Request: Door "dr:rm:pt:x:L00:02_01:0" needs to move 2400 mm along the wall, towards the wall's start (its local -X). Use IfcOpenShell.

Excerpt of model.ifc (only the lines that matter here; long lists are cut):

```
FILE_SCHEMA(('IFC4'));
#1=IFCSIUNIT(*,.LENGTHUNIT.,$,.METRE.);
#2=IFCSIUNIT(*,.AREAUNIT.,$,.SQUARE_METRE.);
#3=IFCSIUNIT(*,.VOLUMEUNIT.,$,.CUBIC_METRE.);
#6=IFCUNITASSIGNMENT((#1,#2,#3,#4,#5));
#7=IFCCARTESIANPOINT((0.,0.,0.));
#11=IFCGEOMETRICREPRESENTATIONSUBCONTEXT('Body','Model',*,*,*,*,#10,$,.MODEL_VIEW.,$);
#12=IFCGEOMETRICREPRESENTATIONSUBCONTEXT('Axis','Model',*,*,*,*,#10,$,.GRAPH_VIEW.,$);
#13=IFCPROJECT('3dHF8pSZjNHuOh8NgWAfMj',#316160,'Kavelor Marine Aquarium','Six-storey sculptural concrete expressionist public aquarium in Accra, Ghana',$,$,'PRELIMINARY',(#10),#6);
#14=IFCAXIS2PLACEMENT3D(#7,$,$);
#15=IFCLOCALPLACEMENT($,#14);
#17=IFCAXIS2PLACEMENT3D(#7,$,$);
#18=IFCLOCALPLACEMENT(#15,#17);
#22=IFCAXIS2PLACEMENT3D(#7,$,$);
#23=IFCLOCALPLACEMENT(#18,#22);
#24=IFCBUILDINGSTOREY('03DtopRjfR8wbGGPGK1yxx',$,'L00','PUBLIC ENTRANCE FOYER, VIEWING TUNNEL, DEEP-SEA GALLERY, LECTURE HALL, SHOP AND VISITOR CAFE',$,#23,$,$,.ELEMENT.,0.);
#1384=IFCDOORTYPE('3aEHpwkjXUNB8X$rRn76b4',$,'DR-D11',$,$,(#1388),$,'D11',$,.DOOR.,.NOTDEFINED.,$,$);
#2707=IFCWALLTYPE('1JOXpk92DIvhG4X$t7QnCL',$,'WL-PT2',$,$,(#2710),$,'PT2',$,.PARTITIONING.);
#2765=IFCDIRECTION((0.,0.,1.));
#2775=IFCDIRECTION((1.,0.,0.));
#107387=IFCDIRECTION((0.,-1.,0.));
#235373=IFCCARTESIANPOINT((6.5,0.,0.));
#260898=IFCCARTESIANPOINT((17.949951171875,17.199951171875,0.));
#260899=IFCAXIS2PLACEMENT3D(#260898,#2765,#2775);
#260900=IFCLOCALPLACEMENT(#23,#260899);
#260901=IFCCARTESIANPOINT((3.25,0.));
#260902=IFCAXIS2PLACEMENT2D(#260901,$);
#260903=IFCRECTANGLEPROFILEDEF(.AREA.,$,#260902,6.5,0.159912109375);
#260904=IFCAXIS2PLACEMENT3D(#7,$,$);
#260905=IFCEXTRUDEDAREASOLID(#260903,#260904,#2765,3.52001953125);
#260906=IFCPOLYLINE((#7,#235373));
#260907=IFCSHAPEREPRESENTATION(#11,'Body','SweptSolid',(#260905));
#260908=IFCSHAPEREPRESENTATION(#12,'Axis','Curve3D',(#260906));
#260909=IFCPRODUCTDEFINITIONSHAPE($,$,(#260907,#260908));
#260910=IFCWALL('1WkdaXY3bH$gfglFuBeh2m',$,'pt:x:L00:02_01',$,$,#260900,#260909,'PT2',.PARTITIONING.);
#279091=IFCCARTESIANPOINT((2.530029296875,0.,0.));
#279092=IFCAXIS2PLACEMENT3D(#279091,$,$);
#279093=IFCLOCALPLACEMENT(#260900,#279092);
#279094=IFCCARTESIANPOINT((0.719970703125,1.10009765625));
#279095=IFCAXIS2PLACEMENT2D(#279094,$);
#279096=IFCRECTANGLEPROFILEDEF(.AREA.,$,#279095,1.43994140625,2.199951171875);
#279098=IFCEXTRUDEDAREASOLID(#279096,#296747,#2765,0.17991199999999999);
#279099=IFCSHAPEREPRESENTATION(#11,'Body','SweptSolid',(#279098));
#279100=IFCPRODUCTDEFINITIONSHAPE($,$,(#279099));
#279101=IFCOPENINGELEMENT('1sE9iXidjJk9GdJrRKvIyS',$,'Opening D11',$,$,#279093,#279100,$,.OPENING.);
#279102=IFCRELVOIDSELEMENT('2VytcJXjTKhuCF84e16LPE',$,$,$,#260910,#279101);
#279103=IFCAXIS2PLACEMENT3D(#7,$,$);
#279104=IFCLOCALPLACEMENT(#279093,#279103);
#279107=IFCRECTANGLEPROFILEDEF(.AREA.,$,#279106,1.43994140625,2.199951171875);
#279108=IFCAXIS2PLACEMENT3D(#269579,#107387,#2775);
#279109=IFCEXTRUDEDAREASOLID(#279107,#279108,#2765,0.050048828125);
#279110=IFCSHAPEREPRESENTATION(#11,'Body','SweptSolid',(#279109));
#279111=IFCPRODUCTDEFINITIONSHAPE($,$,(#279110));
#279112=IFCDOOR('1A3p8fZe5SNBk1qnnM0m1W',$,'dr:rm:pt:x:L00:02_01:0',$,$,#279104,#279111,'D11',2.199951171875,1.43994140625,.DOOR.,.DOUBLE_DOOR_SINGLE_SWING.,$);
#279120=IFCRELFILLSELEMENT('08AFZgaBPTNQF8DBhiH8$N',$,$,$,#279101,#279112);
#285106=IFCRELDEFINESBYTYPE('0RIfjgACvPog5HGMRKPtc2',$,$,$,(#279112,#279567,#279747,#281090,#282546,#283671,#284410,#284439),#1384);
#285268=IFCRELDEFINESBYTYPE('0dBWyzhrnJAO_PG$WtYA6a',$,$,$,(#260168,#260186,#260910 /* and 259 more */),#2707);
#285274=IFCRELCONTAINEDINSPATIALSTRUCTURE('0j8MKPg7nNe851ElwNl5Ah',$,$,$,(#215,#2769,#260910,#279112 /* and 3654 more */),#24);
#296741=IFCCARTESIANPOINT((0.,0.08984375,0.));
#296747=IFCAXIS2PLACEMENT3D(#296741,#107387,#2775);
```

```python
import ifcopenshell
import ifcopenshell.api.geometry
import ifcopenshell.util.placement

model = ifcopenshell.open("model.ifc")

door = model.by_id(279112)
opening = door.FillsVoids[0].RelatingOpeningElement
wall = opening.VoidsElements[0].RelatingBuildingElement

wall_matrix = ifcopenshell.util.placement.get_local_placement(wall.ObjectPlacement)
shift = wall_matrix[:3, 0] * -2.4
before = ifcopenshell.util.placement.get_local_placement(door.ObjectPlacement)[:3, 3].copy()

# The door is placed relative to its opening, so it follows when the opening moves.
matrix = ifcopenshell.util.placement.get_local_placement(opening.ObjectPlacement)
matrix[:3, 3] += shift
ifcopenshell.api.geometry.edit_object_placement(
    model, product=opening, matrix=matrix, is_si=False, should_transform_children=True
)

after = ifcopenshell.util.placement.get_local_placement(door.ObjectPlacement)[:3, 3]
print("door moved by", (after - before).round(3) + 0.0)

model.write("model_v2.ifc")
```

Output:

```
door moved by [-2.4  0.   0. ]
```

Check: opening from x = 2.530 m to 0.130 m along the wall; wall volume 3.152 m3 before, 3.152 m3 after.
